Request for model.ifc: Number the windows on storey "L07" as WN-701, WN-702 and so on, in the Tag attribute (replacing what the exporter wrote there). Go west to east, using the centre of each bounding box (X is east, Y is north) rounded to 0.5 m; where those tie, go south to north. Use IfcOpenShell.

First a look at what the model holds.

```python
import ifcopenshell
import ifcopenshell.util.element
import ifcopenshell.util.placement

model = ifcopenshell.open("model.ifc")
print(model.schema)
storey = next(s for s in model.by_type("IfcBuildingStorey") if s.Name == "L07")
windows = [e for e in ifcopenshell.util.element.get_decomposition(storey) if e.is_a("IfcWindow")]
for e in sorted(windows, key=lambda e: e.id()):
    origin = ifcopenshell.util.placement.get_local_placement(e.ObjectPlacement)[:3, 3]
    print(e.id(), e.Tag, e.Name, origin.round(2) + 0.0, sep=" | ")
```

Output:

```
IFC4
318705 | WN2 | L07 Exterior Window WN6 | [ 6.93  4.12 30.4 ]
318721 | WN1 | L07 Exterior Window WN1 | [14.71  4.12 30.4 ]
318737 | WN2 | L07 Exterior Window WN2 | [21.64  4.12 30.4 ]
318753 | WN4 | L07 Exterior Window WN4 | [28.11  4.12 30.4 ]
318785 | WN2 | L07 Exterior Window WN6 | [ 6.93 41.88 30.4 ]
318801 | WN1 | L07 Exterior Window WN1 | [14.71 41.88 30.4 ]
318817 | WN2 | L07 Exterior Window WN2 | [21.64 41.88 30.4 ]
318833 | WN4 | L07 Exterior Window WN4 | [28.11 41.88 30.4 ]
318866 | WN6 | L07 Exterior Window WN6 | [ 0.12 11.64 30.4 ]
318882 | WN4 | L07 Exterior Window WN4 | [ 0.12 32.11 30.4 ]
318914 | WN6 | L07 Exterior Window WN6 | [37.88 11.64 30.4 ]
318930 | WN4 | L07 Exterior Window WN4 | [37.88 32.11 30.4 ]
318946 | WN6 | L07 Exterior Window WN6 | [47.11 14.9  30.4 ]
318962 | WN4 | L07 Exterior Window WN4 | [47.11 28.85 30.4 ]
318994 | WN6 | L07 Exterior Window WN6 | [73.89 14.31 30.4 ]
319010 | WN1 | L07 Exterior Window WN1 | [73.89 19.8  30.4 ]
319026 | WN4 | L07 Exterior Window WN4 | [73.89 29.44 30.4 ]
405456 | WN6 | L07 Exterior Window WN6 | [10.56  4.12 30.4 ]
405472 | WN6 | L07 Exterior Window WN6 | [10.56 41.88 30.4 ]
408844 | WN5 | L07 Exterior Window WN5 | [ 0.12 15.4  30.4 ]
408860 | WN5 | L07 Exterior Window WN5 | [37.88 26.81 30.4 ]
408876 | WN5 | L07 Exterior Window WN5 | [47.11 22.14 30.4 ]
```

```python
import ifcopenshell
import ifcopenshell.geom
import ifcopenshell.util.element
import ifcopenshell.util.shape

model = ifcopenshell.open("model.ifc")
settings = ifcopenshell.geom.settings()
settings.set("use-world-coords", True)


def centre(element):
    shape = ifcopenshell.geom.create_shape(settings, element)
    return ifcopenshell.util.shape.get_bbox_centroid(shape.geometry)


storey = next(s for s in model.by_type("IfcBuildingStorey") if s.Name == "L07")
windows = [e for e in ifcopenshell.util.element.get_decomposition(storey) if e.is_a("IfcWindow")]

# Insertion points can sit at a corner or the storey origin, so sort by the geometry (in metres).
centres = {e: centre(e) for e in windows}
windows.sort(key=lambda e: (round(centres[e][0] / 0.5), centres[e][1]))

for i, e in enumerate(windows, start=1):
    number = f"WN-7{i:02d}"
    e.Tag = number
    print(e.id(), number)

model.write("model_updated.ifc")
```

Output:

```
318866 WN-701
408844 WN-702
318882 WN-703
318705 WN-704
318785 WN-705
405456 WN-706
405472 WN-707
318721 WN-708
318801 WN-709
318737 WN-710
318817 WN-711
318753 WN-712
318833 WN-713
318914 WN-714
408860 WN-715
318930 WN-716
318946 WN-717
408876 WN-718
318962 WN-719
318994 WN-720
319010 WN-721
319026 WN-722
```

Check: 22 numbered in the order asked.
